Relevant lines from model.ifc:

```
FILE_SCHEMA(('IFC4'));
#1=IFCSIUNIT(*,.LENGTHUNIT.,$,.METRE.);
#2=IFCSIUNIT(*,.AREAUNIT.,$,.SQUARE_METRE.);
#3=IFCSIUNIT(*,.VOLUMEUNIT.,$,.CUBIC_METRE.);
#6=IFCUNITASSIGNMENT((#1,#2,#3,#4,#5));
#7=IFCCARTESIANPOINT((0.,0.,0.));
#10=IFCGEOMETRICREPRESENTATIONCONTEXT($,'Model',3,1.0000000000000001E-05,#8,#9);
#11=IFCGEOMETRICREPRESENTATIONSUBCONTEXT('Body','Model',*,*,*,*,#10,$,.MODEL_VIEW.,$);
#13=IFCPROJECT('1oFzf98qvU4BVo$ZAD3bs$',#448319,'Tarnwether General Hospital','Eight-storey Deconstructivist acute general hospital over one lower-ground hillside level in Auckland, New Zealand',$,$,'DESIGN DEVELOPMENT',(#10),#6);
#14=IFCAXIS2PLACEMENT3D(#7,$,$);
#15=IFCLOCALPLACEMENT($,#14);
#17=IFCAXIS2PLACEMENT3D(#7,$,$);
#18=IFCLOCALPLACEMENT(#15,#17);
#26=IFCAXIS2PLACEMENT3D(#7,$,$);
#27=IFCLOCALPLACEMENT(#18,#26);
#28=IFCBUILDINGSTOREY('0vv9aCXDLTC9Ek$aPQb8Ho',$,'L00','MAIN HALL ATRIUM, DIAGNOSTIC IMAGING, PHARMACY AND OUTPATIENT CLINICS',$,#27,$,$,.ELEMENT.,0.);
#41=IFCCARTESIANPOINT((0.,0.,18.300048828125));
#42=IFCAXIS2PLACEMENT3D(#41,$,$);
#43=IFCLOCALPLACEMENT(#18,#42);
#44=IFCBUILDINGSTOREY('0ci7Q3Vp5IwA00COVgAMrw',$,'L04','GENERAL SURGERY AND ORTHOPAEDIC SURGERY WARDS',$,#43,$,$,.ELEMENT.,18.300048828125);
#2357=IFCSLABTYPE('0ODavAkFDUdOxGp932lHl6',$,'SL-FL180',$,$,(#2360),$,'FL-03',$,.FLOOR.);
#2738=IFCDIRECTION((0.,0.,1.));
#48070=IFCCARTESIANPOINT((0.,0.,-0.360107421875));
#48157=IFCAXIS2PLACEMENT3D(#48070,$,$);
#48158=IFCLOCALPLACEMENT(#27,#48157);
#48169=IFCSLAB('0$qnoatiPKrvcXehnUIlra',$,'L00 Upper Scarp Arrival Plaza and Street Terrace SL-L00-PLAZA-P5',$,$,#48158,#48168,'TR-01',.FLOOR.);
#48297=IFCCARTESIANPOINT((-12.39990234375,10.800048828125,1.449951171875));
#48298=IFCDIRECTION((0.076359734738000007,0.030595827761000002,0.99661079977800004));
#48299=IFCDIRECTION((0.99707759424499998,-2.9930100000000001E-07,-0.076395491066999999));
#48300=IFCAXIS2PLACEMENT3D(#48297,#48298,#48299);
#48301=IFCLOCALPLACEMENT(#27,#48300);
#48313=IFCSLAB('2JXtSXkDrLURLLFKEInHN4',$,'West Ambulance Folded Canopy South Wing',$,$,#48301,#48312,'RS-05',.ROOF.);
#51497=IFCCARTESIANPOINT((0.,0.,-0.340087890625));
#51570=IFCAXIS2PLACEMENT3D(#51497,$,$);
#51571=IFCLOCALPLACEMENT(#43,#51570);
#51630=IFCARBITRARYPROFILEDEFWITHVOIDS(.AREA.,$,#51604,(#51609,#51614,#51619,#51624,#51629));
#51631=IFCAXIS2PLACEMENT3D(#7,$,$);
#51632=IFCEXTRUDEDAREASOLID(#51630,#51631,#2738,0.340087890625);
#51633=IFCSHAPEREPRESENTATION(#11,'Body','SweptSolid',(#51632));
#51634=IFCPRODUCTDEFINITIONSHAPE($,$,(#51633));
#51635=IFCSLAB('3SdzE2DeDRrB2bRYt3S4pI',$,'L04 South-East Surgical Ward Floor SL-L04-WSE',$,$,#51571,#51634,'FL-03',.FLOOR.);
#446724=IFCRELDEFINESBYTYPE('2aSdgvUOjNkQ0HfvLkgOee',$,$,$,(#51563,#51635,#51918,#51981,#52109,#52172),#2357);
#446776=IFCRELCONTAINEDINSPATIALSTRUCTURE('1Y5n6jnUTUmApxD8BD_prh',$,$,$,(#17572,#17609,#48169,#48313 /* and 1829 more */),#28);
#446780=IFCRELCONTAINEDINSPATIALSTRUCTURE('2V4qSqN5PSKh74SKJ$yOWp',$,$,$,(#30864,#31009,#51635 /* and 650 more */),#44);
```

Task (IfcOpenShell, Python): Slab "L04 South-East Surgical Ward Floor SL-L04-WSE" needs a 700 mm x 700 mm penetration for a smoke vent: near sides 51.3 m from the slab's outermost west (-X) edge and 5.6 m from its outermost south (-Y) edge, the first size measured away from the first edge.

```python
import numpy as np
import ifcopenshell
import ifcopenshell.api.feature
import ifcopenshell.api.geometry
import ifcopenshell.api.root
import ifcopenshell.geom
import ifcopenshell.util.placement
import ifcopenshell.util.representation
import ifcopenshell.util.shape
import ifcopenshell.util.unit

model = ifcopenshell.open("model.ifc")
unit_scale = ifcopenshell.util.unit.calculate_unit_scale(model)
settings = ifcopenshell.geom.settings()


def volume(element):
    """Net volume in cubic metres, openings subtracted."""
    shape = ifcopenshell.geom.create_shape(settings, element)
    return ifcopenshell.util.shape.get_volume(shape.geometry)


slab = model.by_id(51635)
before = volume(slab)

# Extent in the slab's own axes, in metres. The edges named are its -X and -Y sides.
slab_shape = ifcopenshell.geom.create_shape(settings, slab)
vertices = ifcopenshell.util.shape.get_vertices(slab_shape.geometry)
x_min, y_min, bottom = vertices.min(axis=0)
top = vertices[:, 2].max()

opening = ifcopenshell.api.root.create_entity(model, ifc_class="IfcOpeningElement", name="Smoke vent opening", predefined_type="OPENING")
context = ifcopenshell.util.representation.get_context(model, "Model", "Body", "MODEL_VIEW")
width, depth = 0.7, 0.7
outline = [(0.0, 0.0), (width, 0.0), (width, depth), (0.0, depth), (0.0, 0.0)]
# Overshoot both faces by 50 mm so the cut is clean.
shape = ifcopenshell.api.geometry.add_slab_representation(
    model, context=context, depth=top - bottom + 0.1, polyline=outline
)
ifcopenshell.api.geometry.assign_representation(model, product=opening, representation=shape)

matrix = ifcopenshell.util.placement.get_local_placement(slab.ObjectPlacement)
matrix[:, 3] = matrix @ np.append(np.array([x_min + 51.3, y_min + 5.6, bottom - 0.05]) / unit_scale, 1.0)
ifcopenshell.api.geometry.edit_object_placement(model, product=opening, matrix=matrix, is_si=False)
ifcopenshell.api.feature.add_feature(model, feature=opening, element=slab)

after = volume(slab)

print(f"slab volume {before:.3f} -> {after:.3f} m3")

model.write("model_v2.ifc")
```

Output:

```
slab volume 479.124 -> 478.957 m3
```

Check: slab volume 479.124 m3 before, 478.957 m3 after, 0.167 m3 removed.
